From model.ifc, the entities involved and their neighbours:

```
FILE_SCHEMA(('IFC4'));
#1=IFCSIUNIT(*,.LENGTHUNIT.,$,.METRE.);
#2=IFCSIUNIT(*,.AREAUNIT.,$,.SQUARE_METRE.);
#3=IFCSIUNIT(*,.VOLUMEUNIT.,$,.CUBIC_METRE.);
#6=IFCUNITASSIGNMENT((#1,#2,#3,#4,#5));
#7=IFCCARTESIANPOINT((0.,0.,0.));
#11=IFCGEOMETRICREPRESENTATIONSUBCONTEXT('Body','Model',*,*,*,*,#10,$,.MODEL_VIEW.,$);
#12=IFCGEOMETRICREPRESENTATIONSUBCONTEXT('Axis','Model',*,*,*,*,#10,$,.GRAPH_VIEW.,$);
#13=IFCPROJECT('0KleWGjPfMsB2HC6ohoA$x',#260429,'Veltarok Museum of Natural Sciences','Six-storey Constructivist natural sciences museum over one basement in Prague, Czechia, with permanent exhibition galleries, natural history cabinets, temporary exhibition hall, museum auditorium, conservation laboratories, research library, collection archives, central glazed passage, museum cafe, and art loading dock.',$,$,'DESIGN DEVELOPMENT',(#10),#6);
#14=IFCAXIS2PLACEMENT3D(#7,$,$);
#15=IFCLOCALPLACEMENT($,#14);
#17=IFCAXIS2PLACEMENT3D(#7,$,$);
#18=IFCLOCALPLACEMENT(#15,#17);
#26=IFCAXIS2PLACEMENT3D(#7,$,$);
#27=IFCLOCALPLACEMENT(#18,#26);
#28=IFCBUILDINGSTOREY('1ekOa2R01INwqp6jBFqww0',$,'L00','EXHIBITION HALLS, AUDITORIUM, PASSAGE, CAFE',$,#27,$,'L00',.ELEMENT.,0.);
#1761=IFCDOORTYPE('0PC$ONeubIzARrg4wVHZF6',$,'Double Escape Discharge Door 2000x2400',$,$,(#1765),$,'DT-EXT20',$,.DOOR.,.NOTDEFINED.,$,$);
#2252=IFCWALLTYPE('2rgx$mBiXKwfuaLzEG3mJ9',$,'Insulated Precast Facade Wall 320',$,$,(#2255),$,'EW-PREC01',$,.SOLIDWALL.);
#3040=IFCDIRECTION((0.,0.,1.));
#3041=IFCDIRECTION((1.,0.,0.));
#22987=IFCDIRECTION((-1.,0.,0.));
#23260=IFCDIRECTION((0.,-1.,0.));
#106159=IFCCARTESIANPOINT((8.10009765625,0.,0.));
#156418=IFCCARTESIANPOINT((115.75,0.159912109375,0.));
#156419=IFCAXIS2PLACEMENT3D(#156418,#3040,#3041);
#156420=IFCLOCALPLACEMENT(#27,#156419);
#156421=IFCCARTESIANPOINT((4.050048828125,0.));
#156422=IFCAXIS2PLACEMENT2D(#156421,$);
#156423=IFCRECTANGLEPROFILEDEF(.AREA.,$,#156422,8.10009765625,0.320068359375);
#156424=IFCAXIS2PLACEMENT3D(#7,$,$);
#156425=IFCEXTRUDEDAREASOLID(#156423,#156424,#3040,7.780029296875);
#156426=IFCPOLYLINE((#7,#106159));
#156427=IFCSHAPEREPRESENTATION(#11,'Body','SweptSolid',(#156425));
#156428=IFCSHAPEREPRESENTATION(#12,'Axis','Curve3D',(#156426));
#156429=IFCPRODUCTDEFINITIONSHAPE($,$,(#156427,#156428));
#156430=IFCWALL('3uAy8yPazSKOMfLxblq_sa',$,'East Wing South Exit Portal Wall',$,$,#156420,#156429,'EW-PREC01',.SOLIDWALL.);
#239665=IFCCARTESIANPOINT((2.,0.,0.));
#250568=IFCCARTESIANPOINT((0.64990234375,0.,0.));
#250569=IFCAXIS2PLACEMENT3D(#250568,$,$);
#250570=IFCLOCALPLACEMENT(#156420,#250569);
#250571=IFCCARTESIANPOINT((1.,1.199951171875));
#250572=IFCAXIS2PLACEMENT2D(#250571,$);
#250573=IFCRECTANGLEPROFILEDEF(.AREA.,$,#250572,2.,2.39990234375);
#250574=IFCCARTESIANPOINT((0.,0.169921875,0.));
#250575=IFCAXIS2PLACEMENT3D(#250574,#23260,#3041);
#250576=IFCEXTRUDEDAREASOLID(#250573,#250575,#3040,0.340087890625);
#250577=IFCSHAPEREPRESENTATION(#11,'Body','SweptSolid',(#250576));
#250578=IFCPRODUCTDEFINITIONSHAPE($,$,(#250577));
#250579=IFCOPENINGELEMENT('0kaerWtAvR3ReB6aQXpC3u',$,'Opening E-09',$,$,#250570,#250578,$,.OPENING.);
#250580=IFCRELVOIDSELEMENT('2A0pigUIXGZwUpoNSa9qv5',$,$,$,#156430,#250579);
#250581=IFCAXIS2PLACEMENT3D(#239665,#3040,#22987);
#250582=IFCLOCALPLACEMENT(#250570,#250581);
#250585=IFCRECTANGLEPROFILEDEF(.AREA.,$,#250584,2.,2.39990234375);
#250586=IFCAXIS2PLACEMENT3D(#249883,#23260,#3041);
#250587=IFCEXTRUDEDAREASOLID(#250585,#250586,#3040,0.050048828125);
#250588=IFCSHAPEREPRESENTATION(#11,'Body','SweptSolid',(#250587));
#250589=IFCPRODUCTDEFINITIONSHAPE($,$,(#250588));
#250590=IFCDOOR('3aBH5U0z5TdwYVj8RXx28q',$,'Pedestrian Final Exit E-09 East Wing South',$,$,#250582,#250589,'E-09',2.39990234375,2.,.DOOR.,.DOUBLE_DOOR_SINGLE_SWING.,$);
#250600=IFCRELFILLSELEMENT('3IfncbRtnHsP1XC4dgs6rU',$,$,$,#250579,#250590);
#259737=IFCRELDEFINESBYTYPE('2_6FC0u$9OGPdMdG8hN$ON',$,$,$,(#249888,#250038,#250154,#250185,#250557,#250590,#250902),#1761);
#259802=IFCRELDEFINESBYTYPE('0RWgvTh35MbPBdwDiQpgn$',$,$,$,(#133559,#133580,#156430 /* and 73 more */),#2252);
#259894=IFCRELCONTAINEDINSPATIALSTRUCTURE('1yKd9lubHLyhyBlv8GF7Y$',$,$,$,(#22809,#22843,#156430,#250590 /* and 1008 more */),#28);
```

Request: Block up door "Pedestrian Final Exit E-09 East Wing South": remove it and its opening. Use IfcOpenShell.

```python
import ifcopenshell
import ifcopenshell.api.feature
import ifcopenshell.api.root
import ifcopenshell.geom
import ifcopenshell.util.shape

model = ifcopenshell.open("model.ifc")
settings = ifcopenshell.geom.settings()


def volume(element):
    """Net volume in cubic metres, openings subtracted."""
    shape = ifcopenshell.geom.create_shape(settings, element)
    return ifcopenshell.util.shape.get_volume(shape.geometry)


door = model.by_guid("3aBH5U0z5TdwYVj8RXx28q")
opening = door.FillsVoids[0].RelatingOpeningElement
wall = opening.VoidsElements[0].RelatingBuildingElement
before = volume(wall)

ifcopenshell.api.root.remove_product(model, product=door)
ifcopenshell.api.feature.remove_feature(model, feature=opening)

after = volume(wall)

print(f"wall volume {before:.3f} -> {after:.3f} m3")

model.write("model-out.ifc")
```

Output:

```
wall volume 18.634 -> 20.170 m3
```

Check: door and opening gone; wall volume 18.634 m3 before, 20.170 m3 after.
